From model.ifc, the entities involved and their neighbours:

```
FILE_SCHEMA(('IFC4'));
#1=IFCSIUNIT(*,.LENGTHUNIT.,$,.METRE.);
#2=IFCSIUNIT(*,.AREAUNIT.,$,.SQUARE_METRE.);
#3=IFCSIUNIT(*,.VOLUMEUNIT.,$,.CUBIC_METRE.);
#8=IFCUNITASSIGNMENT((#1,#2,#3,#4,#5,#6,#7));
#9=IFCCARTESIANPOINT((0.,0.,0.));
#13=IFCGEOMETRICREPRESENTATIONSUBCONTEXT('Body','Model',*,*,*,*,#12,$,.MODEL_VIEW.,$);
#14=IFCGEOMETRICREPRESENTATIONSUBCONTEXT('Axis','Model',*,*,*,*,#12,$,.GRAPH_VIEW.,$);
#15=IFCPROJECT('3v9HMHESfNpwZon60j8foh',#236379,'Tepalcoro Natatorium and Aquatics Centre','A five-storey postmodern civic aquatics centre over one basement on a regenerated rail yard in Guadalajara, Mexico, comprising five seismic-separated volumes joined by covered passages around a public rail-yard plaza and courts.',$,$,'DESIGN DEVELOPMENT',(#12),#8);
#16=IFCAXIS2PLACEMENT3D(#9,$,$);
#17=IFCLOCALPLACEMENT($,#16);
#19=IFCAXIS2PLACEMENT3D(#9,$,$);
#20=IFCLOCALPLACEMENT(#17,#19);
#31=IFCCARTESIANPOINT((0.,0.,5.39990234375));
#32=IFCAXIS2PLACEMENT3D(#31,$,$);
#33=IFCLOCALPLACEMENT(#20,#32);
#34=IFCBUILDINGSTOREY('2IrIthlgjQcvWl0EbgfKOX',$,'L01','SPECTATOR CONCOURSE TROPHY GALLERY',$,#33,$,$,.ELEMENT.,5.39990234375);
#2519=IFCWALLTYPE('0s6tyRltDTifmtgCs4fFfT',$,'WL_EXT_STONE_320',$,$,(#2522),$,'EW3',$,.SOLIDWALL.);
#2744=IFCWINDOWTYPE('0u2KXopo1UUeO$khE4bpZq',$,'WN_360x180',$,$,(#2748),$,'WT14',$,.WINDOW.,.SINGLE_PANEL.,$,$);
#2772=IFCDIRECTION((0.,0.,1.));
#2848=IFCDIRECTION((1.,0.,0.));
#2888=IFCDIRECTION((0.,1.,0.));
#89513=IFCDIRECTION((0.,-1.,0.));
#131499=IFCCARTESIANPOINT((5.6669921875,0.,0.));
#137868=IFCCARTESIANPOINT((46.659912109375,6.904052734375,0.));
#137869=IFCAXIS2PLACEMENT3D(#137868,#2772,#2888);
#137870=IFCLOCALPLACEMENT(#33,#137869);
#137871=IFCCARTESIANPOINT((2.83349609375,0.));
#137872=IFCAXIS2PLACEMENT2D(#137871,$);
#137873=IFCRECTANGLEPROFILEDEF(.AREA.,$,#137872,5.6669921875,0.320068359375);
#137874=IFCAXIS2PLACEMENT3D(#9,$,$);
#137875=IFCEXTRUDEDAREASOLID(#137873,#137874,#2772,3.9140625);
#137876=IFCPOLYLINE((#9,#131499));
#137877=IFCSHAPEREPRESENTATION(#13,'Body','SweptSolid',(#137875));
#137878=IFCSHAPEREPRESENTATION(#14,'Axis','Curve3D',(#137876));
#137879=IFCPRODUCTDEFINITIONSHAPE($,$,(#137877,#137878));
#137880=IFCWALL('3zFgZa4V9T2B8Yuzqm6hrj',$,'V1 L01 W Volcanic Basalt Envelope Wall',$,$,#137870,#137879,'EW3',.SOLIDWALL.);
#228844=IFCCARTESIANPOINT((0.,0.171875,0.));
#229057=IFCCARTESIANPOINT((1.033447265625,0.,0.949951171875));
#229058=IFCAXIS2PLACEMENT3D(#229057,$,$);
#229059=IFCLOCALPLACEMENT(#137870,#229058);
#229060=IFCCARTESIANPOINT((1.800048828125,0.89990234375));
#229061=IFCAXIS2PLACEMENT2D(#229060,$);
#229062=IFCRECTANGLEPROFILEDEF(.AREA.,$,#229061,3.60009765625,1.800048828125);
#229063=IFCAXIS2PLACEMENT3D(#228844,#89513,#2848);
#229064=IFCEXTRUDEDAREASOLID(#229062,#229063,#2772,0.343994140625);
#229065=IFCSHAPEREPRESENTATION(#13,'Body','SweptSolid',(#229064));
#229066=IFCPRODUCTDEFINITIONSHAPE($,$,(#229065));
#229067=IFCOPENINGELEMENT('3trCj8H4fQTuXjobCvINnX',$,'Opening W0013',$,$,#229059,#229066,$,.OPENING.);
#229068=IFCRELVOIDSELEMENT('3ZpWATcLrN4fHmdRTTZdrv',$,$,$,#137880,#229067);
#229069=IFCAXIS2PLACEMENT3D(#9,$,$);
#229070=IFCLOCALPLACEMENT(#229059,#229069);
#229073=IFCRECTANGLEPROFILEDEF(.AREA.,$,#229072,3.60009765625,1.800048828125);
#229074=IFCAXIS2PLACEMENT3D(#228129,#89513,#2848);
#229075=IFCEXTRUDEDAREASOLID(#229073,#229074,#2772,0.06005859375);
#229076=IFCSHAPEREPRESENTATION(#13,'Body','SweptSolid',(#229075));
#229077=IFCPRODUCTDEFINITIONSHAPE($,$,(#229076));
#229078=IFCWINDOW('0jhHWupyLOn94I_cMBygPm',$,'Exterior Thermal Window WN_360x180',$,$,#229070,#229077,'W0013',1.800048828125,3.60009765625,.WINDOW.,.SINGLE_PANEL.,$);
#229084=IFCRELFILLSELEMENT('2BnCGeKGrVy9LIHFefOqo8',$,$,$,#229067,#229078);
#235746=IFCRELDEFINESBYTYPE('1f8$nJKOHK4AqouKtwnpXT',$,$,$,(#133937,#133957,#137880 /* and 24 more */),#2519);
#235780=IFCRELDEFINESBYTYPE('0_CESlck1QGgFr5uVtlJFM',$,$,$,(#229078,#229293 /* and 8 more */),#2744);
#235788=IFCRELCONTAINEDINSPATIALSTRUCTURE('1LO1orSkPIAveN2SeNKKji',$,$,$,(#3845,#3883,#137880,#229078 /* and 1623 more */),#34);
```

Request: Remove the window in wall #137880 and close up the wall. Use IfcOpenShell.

```python
import ifcopenshell
import ifcopenshell.api.feature
import ifcopenshell.api.root
import ifcopenshell.geom
import ifcopenshell.util.shape

model = ifcopenshell.open("model.ifc")
settings = ifcopenshell.geom.settings()


def volume(element):
    """Net volume in cubic metres, openings subtracted."""
    shape = ifcopenshell.geom.create_shape(settings, element)
    return ifcopenshell.util.shape.get_volume(shape.geometry)


window = model.by_id(229078)
opening = window.FillsVoids[0].RelatingOpeningElement
wall = opening.VoidsElements[0].RelatingBuildingElement
before = volume(wall)

ifcopenshell.api.root.remove_product(model, product=window)
ifcopenshell.api.feature.remove_feature(model, feature=opening)

after = volume(wall)

print(f"wall volume {before:.3f} -> {after:.3f} m3")

model.write("model_rev.ifc")
```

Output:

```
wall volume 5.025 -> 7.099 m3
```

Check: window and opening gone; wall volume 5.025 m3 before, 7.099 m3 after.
